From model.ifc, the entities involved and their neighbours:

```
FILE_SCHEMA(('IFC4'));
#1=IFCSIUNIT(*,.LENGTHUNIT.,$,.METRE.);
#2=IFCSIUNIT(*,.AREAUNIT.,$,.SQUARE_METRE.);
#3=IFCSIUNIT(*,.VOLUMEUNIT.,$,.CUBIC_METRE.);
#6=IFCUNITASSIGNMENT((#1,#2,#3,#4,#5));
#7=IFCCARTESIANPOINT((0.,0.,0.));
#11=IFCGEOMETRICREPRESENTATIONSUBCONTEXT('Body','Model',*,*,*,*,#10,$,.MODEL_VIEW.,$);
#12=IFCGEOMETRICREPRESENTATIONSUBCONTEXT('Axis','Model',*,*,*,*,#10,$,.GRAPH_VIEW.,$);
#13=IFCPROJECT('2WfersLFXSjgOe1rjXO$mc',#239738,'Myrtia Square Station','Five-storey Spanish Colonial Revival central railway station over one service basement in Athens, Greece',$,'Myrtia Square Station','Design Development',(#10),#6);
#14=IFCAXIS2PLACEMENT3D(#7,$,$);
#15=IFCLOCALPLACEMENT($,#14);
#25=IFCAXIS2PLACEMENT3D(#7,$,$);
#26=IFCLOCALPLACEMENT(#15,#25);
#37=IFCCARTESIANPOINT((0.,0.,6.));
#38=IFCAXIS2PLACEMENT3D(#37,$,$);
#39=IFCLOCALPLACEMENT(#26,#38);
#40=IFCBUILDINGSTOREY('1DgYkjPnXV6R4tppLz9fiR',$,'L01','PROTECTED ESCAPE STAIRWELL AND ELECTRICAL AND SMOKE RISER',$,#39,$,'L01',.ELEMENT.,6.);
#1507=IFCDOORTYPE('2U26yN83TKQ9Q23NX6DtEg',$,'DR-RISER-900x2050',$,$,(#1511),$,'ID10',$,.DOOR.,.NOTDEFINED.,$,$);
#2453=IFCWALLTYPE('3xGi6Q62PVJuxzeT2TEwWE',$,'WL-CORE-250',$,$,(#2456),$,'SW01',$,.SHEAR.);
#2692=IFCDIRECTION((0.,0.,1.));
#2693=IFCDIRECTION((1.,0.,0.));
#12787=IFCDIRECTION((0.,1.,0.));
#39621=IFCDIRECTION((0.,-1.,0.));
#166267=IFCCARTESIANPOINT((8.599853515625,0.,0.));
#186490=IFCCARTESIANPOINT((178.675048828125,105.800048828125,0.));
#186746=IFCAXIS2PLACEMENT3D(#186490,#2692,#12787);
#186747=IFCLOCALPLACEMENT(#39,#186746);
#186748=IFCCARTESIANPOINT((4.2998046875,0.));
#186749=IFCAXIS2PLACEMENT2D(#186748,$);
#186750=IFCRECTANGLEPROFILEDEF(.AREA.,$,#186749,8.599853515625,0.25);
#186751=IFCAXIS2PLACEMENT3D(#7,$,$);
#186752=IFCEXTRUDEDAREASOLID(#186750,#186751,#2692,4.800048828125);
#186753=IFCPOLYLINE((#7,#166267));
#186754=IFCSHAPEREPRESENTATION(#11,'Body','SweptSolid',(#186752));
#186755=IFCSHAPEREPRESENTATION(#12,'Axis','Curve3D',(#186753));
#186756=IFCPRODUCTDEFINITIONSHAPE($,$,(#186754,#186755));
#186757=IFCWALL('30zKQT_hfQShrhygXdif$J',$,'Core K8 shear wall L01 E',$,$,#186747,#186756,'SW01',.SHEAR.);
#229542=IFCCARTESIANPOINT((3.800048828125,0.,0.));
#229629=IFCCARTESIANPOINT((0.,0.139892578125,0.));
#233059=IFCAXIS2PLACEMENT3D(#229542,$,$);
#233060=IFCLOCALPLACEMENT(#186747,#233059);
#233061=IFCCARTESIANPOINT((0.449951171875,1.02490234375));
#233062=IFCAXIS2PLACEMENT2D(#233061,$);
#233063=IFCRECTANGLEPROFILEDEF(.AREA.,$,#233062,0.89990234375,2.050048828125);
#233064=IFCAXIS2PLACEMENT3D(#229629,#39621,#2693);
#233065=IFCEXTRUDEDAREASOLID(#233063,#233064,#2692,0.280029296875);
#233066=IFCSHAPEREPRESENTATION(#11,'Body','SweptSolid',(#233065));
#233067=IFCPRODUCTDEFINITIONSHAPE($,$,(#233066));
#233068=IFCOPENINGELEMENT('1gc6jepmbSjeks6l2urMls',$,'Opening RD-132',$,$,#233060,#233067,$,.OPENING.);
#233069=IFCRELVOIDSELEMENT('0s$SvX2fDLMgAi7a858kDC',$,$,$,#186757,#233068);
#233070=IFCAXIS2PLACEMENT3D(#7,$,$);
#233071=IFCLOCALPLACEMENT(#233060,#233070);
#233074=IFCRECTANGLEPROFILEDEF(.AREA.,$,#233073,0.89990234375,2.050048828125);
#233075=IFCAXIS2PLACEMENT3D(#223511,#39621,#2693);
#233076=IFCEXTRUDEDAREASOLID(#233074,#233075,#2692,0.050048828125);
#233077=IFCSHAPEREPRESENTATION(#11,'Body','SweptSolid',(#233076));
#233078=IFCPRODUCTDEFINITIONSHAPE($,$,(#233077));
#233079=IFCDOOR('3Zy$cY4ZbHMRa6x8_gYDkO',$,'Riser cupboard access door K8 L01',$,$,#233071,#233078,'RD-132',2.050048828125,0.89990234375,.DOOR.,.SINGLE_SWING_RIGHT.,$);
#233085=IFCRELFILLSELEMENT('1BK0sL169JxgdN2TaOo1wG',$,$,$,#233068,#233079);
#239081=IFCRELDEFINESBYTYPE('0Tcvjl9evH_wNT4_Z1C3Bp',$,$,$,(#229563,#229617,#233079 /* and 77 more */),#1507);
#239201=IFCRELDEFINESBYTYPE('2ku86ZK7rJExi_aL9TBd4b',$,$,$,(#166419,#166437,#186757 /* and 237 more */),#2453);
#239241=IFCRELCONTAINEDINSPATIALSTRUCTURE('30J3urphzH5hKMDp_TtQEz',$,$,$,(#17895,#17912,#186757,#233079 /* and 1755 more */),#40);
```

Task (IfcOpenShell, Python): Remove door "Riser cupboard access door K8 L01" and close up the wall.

```python
import ifcopenshell
import ifcopenshell.api.feature
import ifcopenshell.api.root
import ifcopenshell.geom
import ifcopenshell.util.shape

model = ifcopenshell.open("model.ifc")
settings = ifcopenshell.geom.settings()


def volume(element):
    """Net volume in cubic metres, openings subtracted."""
    shape = ifcopenshell.geom.create_shape(settings, element)
    return ifcopenshell.util.shape.get_volume(shape.geometry)


door = model.by_guid("3Zy$cY4ZbHMRa6x8_gYDkO")
opening = door.FillsVoids[0].RelatingOpeningElement
wall = opening.VoidsElements[0].RelatingBuildingElement
before = volume(wall)

ifcopenshell.api.root.remove_product(model, product=door)
ifcopenshell.api.feature.remove_feature(model, feature=opening)

after = volume(wall)

print(f"wall volume {before:.3f} -> {after:.3f} m3")

model.write("model_edited.ifc")
```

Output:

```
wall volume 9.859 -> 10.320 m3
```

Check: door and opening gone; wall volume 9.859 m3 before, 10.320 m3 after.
